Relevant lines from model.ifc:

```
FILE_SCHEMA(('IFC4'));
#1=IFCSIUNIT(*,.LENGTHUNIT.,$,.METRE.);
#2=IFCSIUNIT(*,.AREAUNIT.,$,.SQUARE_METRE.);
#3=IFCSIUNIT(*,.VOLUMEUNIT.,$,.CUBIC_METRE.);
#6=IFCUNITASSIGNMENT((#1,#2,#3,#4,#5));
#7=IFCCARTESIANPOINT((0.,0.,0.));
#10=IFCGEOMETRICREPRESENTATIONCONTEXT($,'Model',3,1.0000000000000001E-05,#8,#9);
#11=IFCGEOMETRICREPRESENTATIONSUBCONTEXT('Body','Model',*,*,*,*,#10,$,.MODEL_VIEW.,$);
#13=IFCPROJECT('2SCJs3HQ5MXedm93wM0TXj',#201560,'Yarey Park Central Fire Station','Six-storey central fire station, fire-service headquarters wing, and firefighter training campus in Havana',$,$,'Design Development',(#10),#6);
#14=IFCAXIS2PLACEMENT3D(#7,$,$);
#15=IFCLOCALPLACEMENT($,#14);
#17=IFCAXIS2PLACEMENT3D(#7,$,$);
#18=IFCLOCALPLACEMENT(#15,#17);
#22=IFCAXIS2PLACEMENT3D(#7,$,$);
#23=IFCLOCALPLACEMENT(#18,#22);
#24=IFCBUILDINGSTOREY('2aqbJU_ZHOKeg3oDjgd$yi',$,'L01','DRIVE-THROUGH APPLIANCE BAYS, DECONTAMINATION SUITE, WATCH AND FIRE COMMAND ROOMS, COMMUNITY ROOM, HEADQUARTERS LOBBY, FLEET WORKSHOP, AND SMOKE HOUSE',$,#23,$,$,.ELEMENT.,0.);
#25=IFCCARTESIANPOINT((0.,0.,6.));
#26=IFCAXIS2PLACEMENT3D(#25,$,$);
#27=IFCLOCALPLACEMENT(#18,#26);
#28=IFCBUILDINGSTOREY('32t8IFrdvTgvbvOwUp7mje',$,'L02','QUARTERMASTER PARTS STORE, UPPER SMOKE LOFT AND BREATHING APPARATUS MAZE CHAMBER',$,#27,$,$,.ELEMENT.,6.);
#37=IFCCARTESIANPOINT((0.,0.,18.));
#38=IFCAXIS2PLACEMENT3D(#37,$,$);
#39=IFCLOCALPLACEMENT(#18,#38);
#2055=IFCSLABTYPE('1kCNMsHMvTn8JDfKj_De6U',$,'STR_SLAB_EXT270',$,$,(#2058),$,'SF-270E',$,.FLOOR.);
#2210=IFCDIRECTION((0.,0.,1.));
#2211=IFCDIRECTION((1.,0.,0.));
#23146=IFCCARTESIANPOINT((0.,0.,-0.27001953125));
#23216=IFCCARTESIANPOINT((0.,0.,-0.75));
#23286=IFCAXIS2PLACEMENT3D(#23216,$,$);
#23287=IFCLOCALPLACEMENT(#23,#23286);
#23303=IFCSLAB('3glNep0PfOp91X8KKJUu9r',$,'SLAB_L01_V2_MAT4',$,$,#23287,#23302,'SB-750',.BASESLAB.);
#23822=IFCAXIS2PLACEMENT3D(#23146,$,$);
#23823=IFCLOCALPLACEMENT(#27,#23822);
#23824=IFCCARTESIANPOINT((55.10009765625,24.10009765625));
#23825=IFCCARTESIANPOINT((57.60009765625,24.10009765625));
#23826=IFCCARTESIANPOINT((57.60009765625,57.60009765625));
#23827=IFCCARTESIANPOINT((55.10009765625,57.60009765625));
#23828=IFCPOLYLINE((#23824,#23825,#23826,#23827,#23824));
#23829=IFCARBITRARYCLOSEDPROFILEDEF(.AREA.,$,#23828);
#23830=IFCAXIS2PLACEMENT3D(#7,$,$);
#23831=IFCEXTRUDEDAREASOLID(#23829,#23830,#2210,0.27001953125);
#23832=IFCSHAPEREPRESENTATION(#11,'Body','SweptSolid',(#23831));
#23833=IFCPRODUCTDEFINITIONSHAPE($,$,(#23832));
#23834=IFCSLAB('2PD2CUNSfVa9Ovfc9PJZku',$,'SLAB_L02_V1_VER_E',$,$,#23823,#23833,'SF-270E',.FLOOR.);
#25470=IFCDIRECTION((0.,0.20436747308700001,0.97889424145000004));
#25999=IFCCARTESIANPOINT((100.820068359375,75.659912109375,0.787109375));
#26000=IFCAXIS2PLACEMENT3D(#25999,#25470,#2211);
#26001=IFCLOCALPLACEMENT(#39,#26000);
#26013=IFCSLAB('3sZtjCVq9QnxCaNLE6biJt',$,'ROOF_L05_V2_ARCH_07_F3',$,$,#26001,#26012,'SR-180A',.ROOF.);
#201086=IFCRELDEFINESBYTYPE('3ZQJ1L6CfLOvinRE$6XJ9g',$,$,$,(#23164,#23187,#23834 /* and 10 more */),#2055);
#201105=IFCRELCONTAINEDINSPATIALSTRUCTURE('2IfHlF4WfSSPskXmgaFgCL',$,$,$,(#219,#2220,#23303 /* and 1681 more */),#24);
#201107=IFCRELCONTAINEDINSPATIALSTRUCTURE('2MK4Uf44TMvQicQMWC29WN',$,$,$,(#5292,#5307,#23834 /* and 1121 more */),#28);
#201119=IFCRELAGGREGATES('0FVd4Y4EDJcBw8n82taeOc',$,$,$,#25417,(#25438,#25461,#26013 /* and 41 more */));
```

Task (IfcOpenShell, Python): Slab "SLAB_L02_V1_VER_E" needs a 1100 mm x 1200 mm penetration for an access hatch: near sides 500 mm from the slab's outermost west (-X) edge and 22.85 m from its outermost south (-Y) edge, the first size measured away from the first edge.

```python
import numpy as np
import ifcopenshell
import ifcopenshell.api.feature
import ifcopenshell.api.geometry
import ifcopenshell.api.root
import ifcopenshell.geom
import ifcopenshell.util.placement
import ifcopenshell.util.representation
import ifcopenshell.util.shape
import ifcopenshell.util.unit

model = ifcopenshell.open("model.ifc")
unit_scale = ifcopenshell.util.unit.calculate_unit_scale(model)
settings = ifcopenshell.geom.settings()


def volume(element):
    """Net volume in cubic metres, openings subtracted."""
    shape = ifcopenshell.geom.create_shape(settings, element)
    return ifcopenshell.util.shape.get_volume(shape.geometry)


slab = model.by_id(23834)
before = volume(slab)

# Extent in the slab's own axes, in metres. The edges named are its -X and -Y sides.
slab_shape = ifcopenshell.geom.create_shape(settings, slab)
vertices = ifcopenshell.util.shape.get_vertices(slab_shape.geometry)
x_min, y_min, bottom = vertices.min(axis=0)
top = vertices[:, 2].max()

opening = ifcopenshell.api.root.create_entity(model, ifc_class="IfcOpeningElement", name="Access hatch opening", predefined_type="OPENING")
context = ifcopenshell.util.representation.get_context(model, "Model", "Body", "MODEL_VIEW")
width, depth = 1.1, 1.2
outline = [(0.0, 0.0), (width, 0.0), (width, depth), (0.0, depth), (0.0, 0.0)]
# Overshoot both faces by 50 mm so the cut is clean.
shape = ifcopenshell.api.geometry.add_slab_representation(
    model, context=context, depth=top - bottom + 0.1, polyline=outline
)
ifcopenshell.api.geometry.assign_representation(model, product=opening, representation=shape)

matrix = ifcopenshell.util.placement.get_local_placement(slab.ObjectPlacement)
matrix[:, 3] = matrix @ np.append(np.array([x_min + 0.5, y_min + 22.85, bottom - 0.05]) / unit_scale, 1.0)
ifcopenshell.api.geometry.edit_object_placement(model, product=opening, matrix=matrix, is_si=False)
ifcopenshell.api.feature.add_feature(model, feature=opening, element=slab)

after = volume(slab)

print(f"slab volume {before:.3f} -> {after:.3f} m3")

model.write("model_edited.ifc")
```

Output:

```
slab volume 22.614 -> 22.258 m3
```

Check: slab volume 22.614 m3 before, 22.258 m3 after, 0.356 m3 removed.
